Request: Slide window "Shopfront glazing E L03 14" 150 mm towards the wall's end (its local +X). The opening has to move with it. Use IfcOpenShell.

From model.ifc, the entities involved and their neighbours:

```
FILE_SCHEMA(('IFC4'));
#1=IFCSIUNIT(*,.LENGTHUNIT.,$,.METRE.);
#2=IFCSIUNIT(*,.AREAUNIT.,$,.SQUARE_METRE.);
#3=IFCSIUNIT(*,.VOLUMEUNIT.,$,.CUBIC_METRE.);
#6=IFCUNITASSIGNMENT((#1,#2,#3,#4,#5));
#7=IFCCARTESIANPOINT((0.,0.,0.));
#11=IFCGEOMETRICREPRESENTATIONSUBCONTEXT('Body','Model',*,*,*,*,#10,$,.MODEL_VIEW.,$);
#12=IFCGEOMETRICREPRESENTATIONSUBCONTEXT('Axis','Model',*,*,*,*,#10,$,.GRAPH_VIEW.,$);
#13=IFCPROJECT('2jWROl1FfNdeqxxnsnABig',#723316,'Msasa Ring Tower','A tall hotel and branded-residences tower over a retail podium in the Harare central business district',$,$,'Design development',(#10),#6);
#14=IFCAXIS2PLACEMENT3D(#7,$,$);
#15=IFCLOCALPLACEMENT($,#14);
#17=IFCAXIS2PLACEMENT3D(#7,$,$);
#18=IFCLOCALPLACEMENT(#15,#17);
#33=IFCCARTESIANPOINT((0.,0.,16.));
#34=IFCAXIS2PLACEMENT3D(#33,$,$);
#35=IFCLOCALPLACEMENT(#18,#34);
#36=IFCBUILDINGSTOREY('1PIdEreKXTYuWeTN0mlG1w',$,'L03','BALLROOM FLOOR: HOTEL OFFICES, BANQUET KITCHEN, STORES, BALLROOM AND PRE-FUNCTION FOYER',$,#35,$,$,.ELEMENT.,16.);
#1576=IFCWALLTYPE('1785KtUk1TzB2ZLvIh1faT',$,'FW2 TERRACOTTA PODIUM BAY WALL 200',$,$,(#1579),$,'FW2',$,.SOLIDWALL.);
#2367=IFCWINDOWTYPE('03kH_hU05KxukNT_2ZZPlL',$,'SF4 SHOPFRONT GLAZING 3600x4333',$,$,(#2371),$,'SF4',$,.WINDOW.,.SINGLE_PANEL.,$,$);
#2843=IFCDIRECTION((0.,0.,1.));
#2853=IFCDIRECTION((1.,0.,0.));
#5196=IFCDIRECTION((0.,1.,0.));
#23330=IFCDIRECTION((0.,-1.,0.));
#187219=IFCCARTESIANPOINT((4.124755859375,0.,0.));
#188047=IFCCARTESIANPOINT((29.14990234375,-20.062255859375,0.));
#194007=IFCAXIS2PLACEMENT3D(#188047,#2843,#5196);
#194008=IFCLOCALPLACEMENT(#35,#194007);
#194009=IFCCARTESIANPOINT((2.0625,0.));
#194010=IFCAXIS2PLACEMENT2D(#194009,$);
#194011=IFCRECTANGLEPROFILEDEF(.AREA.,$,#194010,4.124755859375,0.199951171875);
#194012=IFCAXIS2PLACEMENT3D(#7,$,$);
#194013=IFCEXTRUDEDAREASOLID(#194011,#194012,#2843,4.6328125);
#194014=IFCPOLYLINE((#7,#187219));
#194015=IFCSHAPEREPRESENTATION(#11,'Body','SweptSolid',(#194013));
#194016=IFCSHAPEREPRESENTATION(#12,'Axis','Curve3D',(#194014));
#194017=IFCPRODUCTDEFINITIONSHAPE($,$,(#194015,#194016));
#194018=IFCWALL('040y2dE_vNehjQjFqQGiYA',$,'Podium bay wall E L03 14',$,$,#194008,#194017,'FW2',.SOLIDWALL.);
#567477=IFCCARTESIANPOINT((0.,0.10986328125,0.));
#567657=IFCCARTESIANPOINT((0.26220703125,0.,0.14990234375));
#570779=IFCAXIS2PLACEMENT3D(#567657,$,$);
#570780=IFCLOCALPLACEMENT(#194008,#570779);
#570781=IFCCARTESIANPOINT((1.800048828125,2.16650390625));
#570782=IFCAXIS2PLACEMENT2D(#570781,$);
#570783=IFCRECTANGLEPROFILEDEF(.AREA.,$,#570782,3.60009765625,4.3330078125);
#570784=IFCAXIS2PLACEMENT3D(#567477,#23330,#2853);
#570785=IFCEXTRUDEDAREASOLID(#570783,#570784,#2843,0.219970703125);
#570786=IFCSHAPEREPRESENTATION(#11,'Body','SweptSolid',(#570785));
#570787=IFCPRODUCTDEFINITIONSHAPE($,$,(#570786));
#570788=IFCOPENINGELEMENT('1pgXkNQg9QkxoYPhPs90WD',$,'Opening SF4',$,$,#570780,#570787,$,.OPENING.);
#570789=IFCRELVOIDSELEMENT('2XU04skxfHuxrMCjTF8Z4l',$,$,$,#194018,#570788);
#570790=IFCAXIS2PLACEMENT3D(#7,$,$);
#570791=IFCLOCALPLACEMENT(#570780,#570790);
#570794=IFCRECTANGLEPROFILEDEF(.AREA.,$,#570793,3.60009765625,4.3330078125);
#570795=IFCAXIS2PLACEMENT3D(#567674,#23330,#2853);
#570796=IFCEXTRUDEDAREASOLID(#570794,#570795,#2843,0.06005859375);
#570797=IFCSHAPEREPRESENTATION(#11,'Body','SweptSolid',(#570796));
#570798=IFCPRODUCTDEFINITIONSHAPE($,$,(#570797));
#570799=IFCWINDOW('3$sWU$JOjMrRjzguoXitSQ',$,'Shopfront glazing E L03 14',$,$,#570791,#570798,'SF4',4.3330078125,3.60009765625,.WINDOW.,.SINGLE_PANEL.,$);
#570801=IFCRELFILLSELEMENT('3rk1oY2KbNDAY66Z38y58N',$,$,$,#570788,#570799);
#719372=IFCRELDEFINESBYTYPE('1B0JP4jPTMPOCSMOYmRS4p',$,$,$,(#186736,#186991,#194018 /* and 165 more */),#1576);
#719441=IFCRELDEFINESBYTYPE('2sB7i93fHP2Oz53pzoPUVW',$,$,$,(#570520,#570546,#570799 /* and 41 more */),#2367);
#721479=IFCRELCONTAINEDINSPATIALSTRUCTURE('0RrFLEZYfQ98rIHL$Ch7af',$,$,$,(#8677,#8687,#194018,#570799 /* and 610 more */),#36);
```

```python
import ifcopenshell
import ifcopenshell.api.geometry
import ifcopenshell.util.placement
import ifcopenshell.util.unit

model = ifcopenshell.open("model.ifc")
unit_scale = ifcopenshell.util.unit.calculate_unit_scale(model)

window = model.by_guid("3$sWU$JOjMrRjzguoXitSQ")
opening = window.FillsVoids[0].RelatingOpeningElement
wall = opening.VoidsElements[0].RelatingBuildingElement

wall_matrix = ifcopenshell.util.placement.get_local_placement(wall.ObjectPlacement)
shift = wall_matrix[:3, 0] * 0.15 / unit_scale
before = ifcopenshell.util.placement.get_local_placement(window.ObjectPlacement)[:3, 3].copy()

# The window is placed relative to its opening, so it follows when the opening moves.
matrix = ifcopenshell.util.placement.get_local_placement(opening.ObjectPlacement)
matrix[:3, 3] += shift
ifcopenshell.api.geometry.edit_object_placement(
    model, product=opening, matrix=matrix, is_si=False, should_transform_children=True
)

after = ifcopenshell.util.placement.get_local_placement(window.ObjectPlacement)[:3, 3]
print("window moved by", (after - before).round(3) + 0.0)

model.write("model-out.ifc")
```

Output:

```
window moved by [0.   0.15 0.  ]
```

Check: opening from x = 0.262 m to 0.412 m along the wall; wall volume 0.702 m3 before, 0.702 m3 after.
